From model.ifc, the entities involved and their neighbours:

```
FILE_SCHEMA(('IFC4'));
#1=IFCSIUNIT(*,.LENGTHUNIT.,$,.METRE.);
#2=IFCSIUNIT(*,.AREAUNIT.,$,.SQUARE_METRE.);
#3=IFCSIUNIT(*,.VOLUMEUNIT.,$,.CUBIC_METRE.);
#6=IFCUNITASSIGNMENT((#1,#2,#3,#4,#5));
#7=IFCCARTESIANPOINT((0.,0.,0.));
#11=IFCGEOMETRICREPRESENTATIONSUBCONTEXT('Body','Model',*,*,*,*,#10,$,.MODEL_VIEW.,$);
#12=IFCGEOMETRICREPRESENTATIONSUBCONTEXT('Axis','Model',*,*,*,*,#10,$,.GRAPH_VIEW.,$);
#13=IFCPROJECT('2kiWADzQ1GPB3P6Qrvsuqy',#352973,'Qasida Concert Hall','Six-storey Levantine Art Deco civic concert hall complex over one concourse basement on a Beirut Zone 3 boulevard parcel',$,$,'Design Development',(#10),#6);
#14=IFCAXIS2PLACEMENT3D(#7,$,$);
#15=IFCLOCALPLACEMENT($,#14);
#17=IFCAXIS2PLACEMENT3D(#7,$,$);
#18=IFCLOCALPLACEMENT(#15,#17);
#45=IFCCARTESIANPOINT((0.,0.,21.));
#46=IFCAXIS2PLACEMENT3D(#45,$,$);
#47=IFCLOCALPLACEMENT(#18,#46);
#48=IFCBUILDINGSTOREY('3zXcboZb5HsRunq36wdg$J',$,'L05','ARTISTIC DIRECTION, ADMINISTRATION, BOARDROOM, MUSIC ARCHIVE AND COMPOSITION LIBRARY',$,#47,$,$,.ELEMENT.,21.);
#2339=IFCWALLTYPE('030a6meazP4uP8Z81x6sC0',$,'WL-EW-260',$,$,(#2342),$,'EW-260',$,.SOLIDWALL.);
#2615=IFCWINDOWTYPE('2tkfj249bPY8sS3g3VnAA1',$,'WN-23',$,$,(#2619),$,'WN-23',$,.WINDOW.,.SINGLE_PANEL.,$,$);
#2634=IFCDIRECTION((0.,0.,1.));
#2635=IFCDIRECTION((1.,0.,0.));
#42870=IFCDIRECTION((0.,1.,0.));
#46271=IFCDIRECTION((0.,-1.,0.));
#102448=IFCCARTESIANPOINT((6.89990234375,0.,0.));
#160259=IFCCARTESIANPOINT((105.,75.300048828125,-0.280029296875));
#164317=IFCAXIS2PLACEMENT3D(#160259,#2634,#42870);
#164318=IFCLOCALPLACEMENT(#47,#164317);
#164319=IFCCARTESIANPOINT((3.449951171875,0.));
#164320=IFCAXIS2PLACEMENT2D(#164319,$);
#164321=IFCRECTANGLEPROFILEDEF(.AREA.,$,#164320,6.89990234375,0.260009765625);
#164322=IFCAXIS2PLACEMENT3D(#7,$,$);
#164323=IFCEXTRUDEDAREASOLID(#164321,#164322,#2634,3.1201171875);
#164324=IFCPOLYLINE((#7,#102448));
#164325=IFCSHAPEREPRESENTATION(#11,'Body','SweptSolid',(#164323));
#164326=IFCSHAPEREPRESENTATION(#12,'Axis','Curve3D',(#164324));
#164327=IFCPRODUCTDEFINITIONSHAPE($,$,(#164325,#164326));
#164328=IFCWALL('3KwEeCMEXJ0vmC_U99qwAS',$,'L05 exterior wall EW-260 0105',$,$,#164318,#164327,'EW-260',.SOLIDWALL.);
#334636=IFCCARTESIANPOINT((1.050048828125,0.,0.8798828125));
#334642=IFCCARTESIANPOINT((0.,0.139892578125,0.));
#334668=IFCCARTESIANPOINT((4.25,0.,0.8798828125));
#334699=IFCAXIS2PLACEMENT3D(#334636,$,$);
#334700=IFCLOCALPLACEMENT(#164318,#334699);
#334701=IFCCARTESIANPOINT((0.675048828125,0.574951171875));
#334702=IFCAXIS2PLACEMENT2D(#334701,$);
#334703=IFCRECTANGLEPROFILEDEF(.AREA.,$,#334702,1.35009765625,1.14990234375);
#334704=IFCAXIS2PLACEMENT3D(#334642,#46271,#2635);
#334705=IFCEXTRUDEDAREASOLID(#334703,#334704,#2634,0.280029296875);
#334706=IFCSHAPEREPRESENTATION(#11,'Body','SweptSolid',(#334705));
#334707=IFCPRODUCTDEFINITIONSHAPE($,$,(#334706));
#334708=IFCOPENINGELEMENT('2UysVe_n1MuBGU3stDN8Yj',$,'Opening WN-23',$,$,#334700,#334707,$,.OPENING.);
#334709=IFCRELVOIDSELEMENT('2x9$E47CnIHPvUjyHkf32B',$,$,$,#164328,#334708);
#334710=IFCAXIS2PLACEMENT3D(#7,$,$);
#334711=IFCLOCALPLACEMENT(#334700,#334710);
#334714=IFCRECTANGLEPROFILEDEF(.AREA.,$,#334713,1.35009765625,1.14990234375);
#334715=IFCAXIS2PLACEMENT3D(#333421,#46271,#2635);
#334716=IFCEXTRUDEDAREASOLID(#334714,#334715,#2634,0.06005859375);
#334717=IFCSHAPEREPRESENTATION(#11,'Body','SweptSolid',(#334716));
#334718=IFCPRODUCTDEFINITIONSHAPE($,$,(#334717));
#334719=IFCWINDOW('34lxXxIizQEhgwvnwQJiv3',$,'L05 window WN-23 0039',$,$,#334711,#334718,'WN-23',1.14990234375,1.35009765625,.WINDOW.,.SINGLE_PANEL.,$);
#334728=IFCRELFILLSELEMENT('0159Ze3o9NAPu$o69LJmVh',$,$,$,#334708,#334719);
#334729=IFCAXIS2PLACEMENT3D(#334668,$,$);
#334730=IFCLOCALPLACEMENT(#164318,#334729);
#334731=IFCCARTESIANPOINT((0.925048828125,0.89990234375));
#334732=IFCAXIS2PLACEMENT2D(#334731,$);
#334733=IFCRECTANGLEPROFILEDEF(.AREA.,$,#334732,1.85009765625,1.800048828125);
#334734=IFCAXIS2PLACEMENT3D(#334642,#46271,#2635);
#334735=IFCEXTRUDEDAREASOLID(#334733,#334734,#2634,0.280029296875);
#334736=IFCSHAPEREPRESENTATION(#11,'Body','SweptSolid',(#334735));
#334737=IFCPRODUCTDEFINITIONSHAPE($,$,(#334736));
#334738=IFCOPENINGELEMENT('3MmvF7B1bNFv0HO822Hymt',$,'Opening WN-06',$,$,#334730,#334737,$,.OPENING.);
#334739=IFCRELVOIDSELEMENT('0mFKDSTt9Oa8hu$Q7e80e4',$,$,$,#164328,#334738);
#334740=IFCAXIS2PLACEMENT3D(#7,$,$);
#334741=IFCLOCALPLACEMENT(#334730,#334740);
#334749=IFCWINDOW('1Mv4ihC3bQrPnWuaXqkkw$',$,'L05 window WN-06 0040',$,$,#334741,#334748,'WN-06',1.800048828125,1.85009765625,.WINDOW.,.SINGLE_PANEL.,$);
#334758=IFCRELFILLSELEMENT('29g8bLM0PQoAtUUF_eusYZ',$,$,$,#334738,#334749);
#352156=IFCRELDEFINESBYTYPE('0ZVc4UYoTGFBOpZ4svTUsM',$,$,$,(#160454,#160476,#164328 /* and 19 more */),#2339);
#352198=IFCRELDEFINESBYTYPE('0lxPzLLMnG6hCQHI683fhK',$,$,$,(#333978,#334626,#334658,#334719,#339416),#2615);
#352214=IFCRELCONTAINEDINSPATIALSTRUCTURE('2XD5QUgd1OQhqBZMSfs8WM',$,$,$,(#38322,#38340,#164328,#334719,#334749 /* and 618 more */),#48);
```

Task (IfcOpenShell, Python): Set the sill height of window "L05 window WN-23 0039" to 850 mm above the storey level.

```python
import numpy as np
import ifcopenshell
import ifcopenshell.api.geometry
import ifcopenshell.geom
import ifcopenshell.util.element
import ifcopenshell.util.placement
import ifcopenshell.util.shape
import ifcopenshell.util.unit

model = ifcopenshell.open("model.ifc")
unit_scale = ifcopenshell.util.unit.calculate_unit_scale(model)

window = model.by_id(334719)
opening = window.FillsVoids[0].RelatingOpeningElement
storey = ifcopenshell.util.element.get_container(window, ifc_class="IfcBuildingStorey")
level = ifcopenshell.util.placement.get_local_placement(storey.ObjectPlacement)[2, 3]

# The opening's origin need not be at the sill, so measure its lowest point.
shape = ifcopenshell.geom.create_shape(ifcopenshell.geom.settings(), opening)
bottom = ifcopenshell.util.shape.get_shape_bottom_elevation(shape, shape.geometry) / unit_scale
dz = level + 0.85 / unit_scale - bottom

shift = np.array([0.0, 0.0, dz])
# The window is placed relative to its opening, so it follows when the opening moves.
matrix = ifcopenshell.util.placement.get_local_placement(opening.ObjectPlacement)
matrix[:3, 3] += shift
ifcopenshell.api.geometry.edit_object_placement(
    model, product=opening, matrix=matrix, is_si=False, should_transform_children=True
)

print(f"moved by {dz * unit_scale:+.3f} m")

model.write("model_edited.ifc")
```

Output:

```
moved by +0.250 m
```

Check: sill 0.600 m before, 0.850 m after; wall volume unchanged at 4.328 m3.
